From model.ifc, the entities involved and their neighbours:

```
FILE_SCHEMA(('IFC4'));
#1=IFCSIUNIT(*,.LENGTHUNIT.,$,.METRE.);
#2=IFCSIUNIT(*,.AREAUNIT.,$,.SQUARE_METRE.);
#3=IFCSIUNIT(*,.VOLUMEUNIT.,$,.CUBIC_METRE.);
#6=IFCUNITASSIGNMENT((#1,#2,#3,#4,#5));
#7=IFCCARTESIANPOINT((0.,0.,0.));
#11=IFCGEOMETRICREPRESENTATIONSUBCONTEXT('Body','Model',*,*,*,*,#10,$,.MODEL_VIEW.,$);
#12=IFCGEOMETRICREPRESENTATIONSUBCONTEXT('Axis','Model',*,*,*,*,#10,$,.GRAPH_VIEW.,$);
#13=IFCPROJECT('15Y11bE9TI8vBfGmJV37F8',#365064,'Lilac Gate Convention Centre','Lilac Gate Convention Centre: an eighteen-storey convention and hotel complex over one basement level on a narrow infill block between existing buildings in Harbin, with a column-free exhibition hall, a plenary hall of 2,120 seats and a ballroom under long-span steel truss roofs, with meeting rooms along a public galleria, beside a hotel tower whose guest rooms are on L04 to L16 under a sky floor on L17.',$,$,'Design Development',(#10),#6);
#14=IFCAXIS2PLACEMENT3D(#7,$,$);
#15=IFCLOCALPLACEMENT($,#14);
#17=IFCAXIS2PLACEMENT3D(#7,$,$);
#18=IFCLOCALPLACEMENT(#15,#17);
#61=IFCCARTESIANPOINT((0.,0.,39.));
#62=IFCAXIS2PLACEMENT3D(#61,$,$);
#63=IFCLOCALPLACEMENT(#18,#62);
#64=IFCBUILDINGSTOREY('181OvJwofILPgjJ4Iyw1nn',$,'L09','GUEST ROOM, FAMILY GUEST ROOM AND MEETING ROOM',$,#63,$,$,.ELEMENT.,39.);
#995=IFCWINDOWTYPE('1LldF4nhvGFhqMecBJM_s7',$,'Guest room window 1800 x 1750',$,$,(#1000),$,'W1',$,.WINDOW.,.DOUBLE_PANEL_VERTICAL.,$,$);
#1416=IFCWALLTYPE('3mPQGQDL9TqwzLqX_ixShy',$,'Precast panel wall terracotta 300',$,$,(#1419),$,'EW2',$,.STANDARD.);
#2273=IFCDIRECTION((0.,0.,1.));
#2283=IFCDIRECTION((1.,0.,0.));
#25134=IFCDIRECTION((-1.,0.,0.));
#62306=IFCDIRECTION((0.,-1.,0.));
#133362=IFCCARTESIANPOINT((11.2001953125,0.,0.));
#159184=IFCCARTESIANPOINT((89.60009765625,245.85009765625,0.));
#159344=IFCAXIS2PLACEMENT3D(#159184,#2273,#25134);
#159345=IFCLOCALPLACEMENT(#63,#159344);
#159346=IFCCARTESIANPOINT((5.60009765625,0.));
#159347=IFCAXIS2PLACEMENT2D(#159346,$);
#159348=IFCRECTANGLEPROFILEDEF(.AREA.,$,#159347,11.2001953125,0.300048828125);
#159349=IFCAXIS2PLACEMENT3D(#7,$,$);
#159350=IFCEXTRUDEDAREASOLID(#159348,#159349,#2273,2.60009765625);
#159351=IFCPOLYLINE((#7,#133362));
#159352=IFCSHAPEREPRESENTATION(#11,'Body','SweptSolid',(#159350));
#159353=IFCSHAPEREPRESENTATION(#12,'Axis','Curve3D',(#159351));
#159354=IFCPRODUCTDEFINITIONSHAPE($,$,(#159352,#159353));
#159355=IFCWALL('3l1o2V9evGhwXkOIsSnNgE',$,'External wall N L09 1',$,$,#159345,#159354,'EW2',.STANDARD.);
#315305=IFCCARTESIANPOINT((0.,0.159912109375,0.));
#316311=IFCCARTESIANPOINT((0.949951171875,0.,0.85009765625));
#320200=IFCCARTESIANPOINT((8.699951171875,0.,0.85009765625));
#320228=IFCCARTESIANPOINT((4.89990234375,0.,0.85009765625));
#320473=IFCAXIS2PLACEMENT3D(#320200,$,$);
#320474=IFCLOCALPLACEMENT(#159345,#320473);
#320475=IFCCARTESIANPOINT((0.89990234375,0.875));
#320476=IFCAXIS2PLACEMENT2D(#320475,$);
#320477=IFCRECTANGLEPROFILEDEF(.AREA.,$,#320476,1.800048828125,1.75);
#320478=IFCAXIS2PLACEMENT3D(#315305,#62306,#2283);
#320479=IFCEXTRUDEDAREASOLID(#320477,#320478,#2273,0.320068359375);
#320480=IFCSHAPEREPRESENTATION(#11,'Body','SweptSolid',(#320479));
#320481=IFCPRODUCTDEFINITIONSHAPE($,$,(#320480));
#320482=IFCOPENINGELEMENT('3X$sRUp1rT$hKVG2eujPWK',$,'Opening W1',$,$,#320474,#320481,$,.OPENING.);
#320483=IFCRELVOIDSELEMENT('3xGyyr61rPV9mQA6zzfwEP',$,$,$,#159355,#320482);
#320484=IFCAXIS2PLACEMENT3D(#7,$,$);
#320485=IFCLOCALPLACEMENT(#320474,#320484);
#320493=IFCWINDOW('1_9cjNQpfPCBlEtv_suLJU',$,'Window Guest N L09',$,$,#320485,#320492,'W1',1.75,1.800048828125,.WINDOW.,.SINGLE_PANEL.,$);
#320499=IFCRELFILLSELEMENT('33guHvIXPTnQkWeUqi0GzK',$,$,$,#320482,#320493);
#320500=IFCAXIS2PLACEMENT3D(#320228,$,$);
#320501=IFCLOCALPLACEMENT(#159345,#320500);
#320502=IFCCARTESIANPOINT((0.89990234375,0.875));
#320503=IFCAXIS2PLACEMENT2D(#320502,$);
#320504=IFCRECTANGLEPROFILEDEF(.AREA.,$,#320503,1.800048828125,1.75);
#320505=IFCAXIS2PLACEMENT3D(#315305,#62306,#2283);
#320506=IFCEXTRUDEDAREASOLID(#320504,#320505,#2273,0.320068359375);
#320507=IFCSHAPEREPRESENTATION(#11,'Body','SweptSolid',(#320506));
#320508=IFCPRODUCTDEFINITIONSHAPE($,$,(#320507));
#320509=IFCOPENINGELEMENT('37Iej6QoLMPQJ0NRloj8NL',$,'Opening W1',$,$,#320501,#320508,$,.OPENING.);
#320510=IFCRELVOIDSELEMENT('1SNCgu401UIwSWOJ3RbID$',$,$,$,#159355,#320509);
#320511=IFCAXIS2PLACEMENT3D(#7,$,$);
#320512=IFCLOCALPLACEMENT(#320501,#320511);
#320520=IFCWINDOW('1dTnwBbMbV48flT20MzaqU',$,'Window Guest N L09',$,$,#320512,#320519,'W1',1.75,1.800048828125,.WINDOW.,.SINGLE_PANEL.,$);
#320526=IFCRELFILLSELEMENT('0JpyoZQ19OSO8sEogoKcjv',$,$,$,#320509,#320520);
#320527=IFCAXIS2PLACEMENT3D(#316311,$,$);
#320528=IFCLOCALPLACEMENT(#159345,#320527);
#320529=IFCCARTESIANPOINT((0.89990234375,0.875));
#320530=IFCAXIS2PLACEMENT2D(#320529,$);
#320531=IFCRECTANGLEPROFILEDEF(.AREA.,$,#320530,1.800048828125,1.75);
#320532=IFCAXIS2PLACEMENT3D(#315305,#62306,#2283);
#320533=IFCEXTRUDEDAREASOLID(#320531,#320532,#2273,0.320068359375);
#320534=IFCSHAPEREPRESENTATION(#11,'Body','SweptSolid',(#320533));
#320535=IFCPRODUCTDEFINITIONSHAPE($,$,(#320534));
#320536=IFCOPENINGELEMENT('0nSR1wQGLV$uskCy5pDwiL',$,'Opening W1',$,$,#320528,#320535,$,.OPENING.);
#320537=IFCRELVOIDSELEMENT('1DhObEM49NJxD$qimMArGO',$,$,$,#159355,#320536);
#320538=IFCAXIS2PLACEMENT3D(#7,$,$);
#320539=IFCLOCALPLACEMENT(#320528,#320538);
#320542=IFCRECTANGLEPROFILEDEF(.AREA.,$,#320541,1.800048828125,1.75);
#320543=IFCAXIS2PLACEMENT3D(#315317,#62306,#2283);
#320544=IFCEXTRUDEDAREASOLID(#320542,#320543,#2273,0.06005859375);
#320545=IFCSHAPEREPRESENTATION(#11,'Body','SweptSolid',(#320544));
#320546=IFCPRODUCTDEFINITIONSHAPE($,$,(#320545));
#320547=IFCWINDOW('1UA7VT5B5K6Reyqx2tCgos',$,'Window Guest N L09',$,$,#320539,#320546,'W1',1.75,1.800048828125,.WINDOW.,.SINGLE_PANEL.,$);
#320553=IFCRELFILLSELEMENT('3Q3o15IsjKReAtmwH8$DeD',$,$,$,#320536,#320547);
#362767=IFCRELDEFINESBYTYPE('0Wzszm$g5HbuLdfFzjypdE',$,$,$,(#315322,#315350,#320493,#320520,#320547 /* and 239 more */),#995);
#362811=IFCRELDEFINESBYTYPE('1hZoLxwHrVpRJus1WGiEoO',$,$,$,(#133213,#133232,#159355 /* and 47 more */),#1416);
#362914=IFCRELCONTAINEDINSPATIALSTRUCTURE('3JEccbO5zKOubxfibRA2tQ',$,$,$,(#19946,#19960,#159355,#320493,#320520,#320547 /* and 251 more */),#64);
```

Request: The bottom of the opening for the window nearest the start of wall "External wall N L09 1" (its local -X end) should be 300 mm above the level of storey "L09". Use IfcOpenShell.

```python
import numpy as np
import ifcopenshell
import ifcopenshell.api.geometry
import ifcopenshell.geom
import ifcopenshell.util.element
import ifcopenshell.util.placement
import ifcopenshell.util.shape
import ifcopenshell.util.unit

model = ifcopenshell.open("model.ifc")
unit_scale = ifcopenshell.util.unit.calculate_unit_scale(model)

window = model.by_guid("1UA7VT5B5K6Reyqx2tCgos")
opening = window.FillsVoids[0].RelatingOpeningElement
storey = ifcopenshell.util.element.get_container(window, ifc_class="IfcBuildingStorey")
level = ifcopenshell.util.placement.get_local_placement(storey.ObjectPlacement)[2, 3]

# The opening's origin need not be at the sill, so measure its lowest point.
shape = ifcopenshell.geom.create_shape(ifcopenshell.geom.settings(), opening)
bottom = ifcopenshell.util.shape.get_shape_bottom_elevation(shape, shape.geometry) / unit_scale
dz = level + 0.3 / unit_scale - bottom

shift = np.array([0.0, 0.0, dz])
# The window is placed relative to its opening, so it follows when the opening moves.
matrix = ifcopenshell.util.placement.get_local_placement(opening.ObjectPlacement)
matrix[:3, 3] += shift
ifcopenshell.api.geometry.edit_object_placement(
    model, product=opening, matrix=matrix, is_si=False, should_transform_children=True
)

print(f"moved by {dz * unit_scale:+.3f} m")

model.write("model_edited.ifc")
```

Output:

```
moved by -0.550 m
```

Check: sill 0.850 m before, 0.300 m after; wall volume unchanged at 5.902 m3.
